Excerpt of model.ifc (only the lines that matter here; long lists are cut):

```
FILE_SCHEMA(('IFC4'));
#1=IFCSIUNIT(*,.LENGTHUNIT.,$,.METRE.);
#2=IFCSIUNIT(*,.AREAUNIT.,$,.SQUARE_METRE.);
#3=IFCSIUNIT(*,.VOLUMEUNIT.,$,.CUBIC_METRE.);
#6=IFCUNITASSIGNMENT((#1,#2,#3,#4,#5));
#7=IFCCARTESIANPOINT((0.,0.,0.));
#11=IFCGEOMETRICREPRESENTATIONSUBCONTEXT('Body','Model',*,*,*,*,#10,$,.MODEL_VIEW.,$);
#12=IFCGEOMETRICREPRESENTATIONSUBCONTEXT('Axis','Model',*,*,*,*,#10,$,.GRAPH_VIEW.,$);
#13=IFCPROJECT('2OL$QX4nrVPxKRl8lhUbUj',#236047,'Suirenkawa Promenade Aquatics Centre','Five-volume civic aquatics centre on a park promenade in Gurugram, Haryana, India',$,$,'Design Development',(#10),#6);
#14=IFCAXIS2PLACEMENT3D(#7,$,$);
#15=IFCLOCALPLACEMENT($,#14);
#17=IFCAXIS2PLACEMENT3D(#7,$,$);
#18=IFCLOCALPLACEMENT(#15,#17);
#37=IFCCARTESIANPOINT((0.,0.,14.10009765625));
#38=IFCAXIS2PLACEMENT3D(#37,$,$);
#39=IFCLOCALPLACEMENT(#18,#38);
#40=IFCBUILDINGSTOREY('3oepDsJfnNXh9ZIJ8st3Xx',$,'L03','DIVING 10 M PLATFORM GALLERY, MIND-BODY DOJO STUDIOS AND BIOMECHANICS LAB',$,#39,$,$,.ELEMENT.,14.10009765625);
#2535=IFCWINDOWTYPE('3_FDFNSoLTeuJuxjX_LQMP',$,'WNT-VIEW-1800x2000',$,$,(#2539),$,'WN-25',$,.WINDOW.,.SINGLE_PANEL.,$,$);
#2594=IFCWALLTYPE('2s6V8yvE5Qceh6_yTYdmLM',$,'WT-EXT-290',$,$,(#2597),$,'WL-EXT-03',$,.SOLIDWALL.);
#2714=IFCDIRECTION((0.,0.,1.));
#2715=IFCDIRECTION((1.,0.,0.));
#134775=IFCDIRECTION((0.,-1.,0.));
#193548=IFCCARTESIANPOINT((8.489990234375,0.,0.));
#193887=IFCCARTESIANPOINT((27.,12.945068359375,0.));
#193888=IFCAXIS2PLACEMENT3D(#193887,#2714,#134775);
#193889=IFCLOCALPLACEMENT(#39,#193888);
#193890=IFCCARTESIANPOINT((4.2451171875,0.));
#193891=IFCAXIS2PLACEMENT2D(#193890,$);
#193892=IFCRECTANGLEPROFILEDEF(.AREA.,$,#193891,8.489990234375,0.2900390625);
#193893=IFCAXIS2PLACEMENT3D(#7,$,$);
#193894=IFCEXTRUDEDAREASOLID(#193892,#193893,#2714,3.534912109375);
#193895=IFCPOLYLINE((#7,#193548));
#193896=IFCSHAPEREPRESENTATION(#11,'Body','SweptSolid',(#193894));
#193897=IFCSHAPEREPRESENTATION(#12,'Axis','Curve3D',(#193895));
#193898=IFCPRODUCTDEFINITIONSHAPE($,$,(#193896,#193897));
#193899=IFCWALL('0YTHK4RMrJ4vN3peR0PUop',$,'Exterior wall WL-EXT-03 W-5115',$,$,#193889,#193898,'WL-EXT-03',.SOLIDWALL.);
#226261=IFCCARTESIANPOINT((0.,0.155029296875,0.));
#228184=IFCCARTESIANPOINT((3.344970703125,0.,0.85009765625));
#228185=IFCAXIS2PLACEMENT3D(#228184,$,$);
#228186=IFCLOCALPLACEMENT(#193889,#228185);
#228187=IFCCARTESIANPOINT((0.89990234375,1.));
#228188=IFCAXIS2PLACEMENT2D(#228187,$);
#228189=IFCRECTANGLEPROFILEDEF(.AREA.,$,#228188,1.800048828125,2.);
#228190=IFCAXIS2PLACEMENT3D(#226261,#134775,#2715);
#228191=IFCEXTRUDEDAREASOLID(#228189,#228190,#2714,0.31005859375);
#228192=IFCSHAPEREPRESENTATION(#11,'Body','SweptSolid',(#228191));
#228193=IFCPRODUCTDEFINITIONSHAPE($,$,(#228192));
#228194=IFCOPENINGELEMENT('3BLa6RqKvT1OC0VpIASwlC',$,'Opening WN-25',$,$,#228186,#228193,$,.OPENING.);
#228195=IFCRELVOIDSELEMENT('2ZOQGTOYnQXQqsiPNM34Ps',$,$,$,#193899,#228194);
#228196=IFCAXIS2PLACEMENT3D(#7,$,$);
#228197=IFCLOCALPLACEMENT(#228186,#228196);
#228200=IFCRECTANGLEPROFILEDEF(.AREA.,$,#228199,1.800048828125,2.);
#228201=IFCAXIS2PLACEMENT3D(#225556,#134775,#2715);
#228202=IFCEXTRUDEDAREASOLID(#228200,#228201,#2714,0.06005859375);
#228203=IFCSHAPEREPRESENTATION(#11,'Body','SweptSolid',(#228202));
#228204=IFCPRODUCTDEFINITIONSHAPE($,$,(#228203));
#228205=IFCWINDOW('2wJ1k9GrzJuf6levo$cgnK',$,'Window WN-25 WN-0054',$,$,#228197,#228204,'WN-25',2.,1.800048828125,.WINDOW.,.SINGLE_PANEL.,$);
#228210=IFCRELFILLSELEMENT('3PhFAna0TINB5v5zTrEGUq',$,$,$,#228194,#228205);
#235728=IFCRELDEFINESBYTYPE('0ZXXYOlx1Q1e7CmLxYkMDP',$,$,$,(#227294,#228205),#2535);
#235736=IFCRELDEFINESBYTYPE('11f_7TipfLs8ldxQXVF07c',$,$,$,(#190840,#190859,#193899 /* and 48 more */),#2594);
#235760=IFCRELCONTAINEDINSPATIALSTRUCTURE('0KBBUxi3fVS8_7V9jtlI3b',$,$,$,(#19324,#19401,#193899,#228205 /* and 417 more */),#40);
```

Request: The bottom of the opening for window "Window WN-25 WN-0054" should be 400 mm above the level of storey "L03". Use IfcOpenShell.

```python
import numpy as np
import ifcopenshell
import ifcopenshell.api.geometry
import ifcopenshell.geom
import ifcopenshell.util.element
import ifcopenshell.util.placement
import ifcopenshell.util.shape
import ifcopenshell.util.unit

model = ifcopenshell.open("model.ifc")
unit_scale = ifcopenshell.util.unit.calculate_unit_scale(model)

window = model.by_guid("2wJ1k9GrzJuf6levo$cgnK")
opening = window.FillsVoids[0].RelatingOpeningElement
storey = ifcopenshell.util.element.get_container(window, ifc_class="IfcBuildingStorey")
level = ifcopenshell.util.placement.get_local_placement(storey.ObjectPlacement)[2, 3]

# The opening's origin need not be at the sill, so measure its lowest point.
shape = ifcopenshell.geom.create_shape(ifcopenshell.geom.settings(), opening)
bottom = ifcopenshell.util.shape.get_shape_bottom_elevation(shape, shape.geometry) / unit_scale
dz = level + 0.4 / unit_scale - bottom

shift = np.array([0.0, 0.0, dz])
# The window is placed relative to its opening, so it follows when the opening moves.
matrix = ifcopenshell.util.placement.get_local_placement(opening.ObjectPlacement)
matrix[:3, 3] += shift
ifcopenshell.api.geometry.edit_object_placement(
    model, product=opening, matrix=matrix, is_si=False, should_transform_children=True
)

print(f"moved by {dz * unit_scale:+.3f} m")

model.write("model_updated.ifc")
```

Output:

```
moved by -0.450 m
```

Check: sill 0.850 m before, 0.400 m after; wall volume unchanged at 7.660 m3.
